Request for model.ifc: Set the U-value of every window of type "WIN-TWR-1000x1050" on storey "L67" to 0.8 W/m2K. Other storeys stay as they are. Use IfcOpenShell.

First a look at what the model holds.

```python
import ifcopenshell
import ifcopenshell.util.element

model = ifcopenshell.open("model.ifc")
print(model.schema)
storey = next(s for s in model.by_type("IfcBuildingStorey") if s.Name == "L67")
windows = [e for e in ifcopenshell.util.element.get_decomposition(storey) if e.is_a("IfcWindow")]
seen = {}
for e in windows:
    element_type = ifcopenshell.util.element.get_type(e)
    key = (element_type.Name if element_type != e and element_type else None, ifcopenshell.util.element.get_pset(e, "Pset_WindowCommon", "ThermalTransmittance"))
    seen[key] = seen.get(key, 0) + 1
for (name, value), count in sorted(seen.items(), key=str):
    print(count, "x", name, "|", value)
```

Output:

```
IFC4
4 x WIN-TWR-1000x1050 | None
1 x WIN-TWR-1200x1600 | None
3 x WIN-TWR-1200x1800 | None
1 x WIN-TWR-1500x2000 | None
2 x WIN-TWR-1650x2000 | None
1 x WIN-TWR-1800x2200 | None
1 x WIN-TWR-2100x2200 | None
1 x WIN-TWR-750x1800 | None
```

```python
import ifcopenshell
import ifcopenshell.api.pset
import ifcopenshell.util.element

model = ifcopenshell.open("model.ifc")

storey = next(s for s in model.by_type("IfcBuildingStorey") if s.Name == "L67")
windows = [e for e in ifcopenshell.util.element.get_decomposition(storey) if e.is_a("IfcWindow")]

count = 0
for e in windows:
    element_type = ifcopenshell.util.element.get_type(e)
    if element_type in (None, e) or element_type.Name != "WIN-TWR-1000x1050":
        continue
    found = ifcopenshell.util.element.get_pset(e, "Pset_WindowCommon", should_inherit=False)
    if found:
        pset = model.by_id(found["id"])
        if len(ifcopenshell.util.element.get_elements_by_pset(pset)) > 1:
            pset = ifcopenshell.api.pset.unshare_pset(model, products=[e], pset=pset)[0]
    else:
        pset = ifcopenshell.api.pset.add_pset(model, product=e, name="Pset_WindowCommon")
    ifcopenshell.api.pset.edit_pset(model, pset=pset, properties={"ThermalTransmittance": 0.8})
    count += 1

print(count, "windows updated")

model.write("model_edited.ifc")
```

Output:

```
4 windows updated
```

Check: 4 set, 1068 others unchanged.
